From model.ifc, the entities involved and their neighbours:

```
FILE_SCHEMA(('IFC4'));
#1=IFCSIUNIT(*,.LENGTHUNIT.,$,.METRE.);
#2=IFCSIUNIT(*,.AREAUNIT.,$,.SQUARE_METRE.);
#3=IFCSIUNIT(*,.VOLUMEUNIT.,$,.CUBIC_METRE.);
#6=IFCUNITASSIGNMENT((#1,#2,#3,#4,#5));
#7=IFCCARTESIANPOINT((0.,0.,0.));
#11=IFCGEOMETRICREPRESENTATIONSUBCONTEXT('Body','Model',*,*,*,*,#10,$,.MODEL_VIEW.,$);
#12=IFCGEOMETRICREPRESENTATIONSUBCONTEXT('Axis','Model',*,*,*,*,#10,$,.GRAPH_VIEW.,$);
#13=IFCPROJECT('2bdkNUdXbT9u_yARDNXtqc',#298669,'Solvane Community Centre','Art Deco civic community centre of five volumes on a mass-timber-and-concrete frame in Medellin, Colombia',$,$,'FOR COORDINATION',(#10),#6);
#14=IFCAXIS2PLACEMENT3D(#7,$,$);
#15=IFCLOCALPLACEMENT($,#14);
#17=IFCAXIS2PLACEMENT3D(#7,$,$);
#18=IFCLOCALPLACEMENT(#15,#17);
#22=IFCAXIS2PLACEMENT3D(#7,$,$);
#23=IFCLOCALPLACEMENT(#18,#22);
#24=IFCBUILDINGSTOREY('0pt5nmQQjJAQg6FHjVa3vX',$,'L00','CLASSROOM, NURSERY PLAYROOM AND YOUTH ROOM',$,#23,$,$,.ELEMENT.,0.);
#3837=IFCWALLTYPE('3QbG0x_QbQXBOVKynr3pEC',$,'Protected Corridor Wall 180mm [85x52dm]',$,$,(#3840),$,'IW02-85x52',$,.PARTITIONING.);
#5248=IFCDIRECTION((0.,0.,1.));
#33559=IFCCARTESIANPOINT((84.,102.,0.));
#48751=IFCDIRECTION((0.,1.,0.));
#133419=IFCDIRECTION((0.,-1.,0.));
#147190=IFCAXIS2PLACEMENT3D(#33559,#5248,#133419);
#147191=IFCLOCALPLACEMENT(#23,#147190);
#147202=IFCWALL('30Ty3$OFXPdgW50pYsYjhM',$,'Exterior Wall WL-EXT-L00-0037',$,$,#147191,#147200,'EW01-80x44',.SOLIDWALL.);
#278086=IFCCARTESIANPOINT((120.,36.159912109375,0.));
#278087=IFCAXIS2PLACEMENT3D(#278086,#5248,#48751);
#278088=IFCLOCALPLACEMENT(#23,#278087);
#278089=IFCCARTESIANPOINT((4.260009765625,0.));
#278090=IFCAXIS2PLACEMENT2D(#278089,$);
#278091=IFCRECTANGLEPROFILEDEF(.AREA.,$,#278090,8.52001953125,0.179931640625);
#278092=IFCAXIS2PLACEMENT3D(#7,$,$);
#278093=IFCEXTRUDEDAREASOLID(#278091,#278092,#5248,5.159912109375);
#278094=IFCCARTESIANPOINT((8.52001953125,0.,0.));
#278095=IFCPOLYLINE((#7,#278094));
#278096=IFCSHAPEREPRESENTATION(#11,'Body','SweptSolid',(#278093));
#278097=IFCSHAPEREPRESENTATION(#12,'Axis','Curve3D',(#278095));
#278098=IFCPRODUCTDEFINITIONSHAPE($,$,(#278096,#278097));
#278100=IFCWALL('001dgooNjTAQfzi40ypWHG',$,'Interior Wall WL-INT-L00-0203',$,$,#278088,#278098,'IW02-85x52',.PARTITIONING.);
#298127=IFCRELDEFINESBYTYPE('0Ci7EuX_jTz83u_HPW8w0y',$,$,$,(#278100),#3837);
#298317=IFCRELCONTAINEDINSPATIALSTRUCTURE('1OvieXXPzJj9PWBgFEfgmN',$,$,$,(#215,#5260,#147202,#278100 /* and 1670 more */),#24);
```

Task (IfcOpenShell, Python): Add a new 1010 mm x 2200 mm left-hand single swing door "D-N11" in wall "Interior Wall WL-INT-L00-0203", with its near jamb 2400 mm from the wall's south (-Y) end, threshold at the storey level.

```python
import numpy as np
import ifcopenshell
import ifcopenshell.api.feature
import ifcopenshell.api.geometry
import ifcopenshell.api.root
import ifcopenshell.api.spatial
import ifcopenshell.geom
import ifcopenshell.util.element
import ifcopenshell.util.placement
import ifcopenshell.util.representation
import ifcopenshell.util.shape
import ifcopenshell.util.unit

model = ifcopenshell.open("model.ifc")
unit_scale = ifcopenshell.util.unit.calculate_unit_scale(model)
settings = ifcopenshell.geom.settings()


def volume(element):
    """Net volume in cubic metres, openings subtracted."""
    shape = ifcopenshell.geom.create_shape(settings, element)
    return ifcopenshell.util.shape.get_volume(shape.geometry)


wall = model.by_id(278100)
storey = ifcopenshell.util.element.get_container(wall, ifc_class="IfcBuildingStorey")
context = ifcopenshell.util.representation.get_context(model, "Model", "Body", "MODEL_VIEW")
before = volume(wall)

width, height, from_end, sill = 1.01, 2.2, 2.4, 0.0  # metres

# The wall runs along its own X axis, and the end named is its -X end.
wall_shape = ifcopenshell.geom.create_shape(settings, wall)
x, y, z = ifcopenshell.util.shape.get_vertices(wall_shape.geometry).T
start = x.min() + from_end
face, thickness = float(y.min()), float(y.max() - y.min())
wall_matrix = ifcopenshell.util.placement.get_local_placement(wall.ObjectPlacement)
level = ifcopenshell.util.placement.get_local_placement(storey.ObjectPlacement)[2, 3]


def in_wall(x, y):
    """Placement at x, y metres in the wall's axes, at sill height."""
    matrix = wall_matrix.copy()
    matrix[:, 3] = wall_matrix @ np.array([x / unit_scale, y / unit_scale, 0.0, 1.0])
    matrix[2, 3] = level + sill / unit_scale
    return matrix


# Opening: a box that overshoots both wall faces by 50 mm.
opening = ifcopenshell.api.root.create_entity(model, ifc_class="IfcOpeningElement", predefined_type="OPENING")
box = ifcopenshell.api.geometry.add_wall_representation(
    model, context=context, length=width, height=height, thickness=thickness + 0.1
)
ifcopenshell.api.geometry.assign_representation(model, product=opening, representation=box)
ifcopenshell.api.geometry.edit_object_placement(model, product=opening, matrix=in_wall(start, face - 0.05), is_si=False)
ifcopenshell.api.feature.add_feature(model, feature=opening, element=wall)

door = ifcopenshell.api.root.create_entity(model, ifc_class="IfcDoor", name="D-N11", predefined_type="DOOR")
door.OverallWidth, door.OverallHeight = width / unit_scale, height / unit_scale
door.OperationType = "SINGLE_SWING_LEFT"
body = ifcopenshell.api.geometry.add_door_representation(
    model,
    context=context,
    overall_width=door.OverallWidth,
    overall_height=door.OverallHeight,
    operation_type="SINGLE_SWING_LEFT",
    lining_properties={"LiningDepth": thickness / unit_scale, "ThresholdDepth": thickness / unit_scale},
)
ifcopenshell.api.geometry.assign_representation(model, product=door, representation=body)
ifcopenshell.api.spatial.assign_container(model, products=[door], relating_structure=storey)
ifcopenshell.api.feature.add_filling(model, opening=opening, element=door)

# The lining spans the wall, so the door starts at the wall face.
ifcopenshell.api.geometry.edit_object_placement(model, product=door, matrix=in_wall(start, face), is_si=False)

after = volume(wall)

print(f"wall volume {before:.3f} -> {after:.3f} m3")

model.write("model_v2.ifc")
```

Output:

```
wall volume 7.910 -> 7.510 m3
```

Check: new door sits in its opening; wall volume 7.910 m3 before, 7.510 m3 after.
